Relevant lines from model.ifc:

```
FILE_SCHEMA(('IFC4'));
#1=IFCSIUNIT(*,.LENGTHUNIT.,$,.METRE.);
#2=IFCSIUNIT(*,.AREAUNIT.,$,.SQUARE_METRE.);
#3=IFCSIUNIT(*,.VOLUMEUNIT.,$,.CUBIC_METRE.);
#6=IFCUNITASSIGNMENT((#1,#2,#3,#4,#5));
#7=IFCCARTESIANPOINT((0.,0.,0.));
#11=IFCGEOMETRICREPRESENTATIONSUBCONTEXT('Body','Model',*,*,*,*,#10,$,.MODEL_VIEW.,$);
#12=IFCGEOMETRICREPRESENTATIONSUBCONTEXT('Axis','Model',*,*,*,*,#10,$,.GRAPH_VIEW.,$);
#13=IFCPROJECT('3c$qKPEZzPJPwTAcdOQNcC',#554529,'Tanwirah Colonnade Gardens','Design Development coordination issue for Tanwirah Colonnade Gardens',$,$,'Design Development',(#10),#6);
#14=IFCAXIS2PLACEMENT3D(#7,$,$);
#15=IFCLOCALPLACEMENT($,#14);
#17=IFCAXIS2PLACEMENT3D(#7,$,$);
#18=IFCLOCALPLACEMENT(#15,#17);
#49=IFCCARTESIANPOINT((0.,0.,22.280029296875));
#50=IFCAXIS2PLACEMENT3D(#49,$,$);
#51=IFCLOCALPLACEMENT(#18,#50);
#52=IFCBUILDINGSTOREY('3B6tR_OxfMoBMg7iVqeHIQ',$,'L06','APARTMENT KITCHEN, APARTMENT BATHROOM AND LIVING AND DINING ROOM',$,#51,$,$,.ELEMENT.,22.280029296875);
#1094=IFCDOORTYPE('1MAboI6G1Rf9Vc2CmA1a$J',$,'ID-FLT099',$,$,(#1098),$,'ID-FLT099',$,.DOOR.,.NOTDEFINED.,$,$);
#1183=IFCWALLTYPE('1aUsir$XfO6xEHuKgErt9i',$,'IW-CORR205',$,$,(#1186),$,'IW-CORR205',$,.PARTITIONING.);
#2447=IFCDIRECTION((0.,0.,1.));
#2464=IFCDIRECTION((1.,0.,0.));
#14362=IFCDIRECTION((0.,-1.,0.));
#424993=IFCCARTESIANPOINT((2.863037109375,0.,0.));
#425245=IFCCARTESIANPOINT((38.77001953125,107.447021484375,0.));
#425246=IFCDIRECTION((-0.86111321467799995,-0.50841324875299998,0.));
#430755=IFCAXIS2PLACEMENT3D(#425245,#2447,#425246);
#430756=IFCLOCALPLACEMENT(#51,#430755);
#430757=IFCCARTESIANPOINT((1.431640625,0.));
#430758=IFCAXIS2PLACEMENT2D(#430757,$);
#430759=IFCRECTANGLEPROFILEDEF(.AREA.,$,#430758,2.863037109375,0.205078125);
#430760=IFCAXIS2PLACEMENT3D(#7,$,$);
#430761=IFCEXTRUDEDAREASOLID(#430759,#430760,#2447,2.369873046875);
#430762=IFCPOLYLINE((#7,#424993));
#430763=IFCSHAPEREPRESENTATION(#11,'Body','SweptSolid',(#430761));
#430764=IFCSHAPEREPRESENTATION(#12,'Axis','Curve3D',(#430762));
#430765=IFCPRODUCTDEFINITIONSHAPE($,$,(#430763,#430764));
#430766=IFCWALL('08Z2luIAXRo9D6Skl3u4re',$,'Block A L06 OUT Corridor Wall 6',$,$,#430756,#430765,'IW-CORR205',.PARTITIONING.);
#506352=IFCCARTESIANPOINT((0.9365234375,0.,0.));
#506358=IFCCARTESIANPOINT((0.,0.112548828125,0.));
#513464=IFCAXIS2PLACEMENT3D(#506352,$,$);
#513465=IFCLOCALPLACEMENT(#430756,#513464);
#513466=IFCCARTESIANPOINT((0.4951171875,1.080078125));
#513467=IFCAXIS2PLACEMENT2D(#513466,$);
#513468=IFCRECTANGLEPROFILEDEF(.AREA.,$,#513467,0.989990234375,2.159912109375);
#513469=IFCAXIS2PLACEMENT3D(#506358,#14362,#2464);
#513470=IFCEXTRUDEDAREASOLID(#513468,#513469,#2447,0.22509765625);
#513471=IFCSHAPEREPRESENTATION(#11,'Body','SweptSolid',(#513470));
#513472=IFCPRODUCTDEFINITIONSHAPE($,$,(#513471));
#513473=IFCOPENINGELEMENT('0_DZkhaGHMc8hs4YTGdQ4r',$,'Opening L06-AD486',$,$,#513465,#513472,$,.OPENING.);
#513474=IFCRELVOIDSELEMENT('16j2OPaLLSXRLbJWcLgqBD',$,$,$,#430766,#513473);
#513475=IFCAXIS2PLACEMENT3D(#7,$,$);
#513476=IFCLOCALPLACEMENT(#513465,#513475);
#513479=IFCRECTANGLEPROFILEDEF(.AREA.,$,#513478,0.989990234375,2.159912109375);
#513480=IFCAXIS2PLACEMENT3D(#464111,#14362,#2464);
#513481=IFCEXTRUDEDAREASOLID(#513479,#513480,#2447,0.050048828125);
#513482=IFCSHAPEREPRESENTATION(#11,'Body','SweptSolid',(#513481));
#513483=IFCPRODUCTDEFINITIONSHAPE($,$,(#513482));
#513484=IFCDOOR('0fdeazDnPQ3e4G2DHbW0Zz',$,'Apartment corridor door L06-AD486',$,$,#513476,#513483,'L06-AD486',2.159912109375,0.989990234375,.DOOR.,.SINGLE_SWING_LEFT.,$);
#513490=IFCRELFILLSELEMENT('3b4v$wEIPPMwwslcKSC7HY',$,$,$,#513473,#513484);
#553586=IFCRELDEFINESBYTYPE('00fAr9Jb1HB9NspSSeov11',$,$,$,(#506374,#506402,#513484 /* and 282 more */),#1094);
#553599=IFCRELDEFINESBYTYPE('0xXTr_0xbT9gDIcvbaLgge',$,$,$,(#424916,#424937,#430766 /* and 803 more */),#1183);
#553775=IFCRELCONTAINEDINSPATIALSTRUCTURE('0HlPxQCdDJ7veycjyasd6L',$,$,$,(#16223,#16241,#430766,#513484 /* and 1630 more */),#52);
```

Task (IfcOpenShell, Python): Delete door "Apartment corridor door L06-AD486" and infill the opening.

```python
import ifcopenshell
import ifcopenshell.api.feature
import ifcopenshell.api.root
import ifcopenshell.geom
import ifcopenshell.util.shape

model = ifcopenshell.open("model.ifc")
settings = ifcopenshell.geom.settings()


def volume(element):
    """Net volume in cubic metres, openings subtracted."""
    shape = ifcopenshell.geom.create_shape(settings, element)
    return ifcopenshell.util.shape.get_volume(shape.geometry)


door = model.by_id(513484)
opening = door.FillsVoids[0].RelatingOpeningElement
wall = opening.VoidsElements[0].RelatingBuildingElement
before = volume(wall)

ifcopenshell.api.root.remove_product(model, product=door)
ifcopenshell.api.feature.remove_feature(model, feature=opening)

after = volume(wall)

print(f"wall volume {before:.3f} -> {after:.3f} m3")

model.write("model_rev.ifc")
```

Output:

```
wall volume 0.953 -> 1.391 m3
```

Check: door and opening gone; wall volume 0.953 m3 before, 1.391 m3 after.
